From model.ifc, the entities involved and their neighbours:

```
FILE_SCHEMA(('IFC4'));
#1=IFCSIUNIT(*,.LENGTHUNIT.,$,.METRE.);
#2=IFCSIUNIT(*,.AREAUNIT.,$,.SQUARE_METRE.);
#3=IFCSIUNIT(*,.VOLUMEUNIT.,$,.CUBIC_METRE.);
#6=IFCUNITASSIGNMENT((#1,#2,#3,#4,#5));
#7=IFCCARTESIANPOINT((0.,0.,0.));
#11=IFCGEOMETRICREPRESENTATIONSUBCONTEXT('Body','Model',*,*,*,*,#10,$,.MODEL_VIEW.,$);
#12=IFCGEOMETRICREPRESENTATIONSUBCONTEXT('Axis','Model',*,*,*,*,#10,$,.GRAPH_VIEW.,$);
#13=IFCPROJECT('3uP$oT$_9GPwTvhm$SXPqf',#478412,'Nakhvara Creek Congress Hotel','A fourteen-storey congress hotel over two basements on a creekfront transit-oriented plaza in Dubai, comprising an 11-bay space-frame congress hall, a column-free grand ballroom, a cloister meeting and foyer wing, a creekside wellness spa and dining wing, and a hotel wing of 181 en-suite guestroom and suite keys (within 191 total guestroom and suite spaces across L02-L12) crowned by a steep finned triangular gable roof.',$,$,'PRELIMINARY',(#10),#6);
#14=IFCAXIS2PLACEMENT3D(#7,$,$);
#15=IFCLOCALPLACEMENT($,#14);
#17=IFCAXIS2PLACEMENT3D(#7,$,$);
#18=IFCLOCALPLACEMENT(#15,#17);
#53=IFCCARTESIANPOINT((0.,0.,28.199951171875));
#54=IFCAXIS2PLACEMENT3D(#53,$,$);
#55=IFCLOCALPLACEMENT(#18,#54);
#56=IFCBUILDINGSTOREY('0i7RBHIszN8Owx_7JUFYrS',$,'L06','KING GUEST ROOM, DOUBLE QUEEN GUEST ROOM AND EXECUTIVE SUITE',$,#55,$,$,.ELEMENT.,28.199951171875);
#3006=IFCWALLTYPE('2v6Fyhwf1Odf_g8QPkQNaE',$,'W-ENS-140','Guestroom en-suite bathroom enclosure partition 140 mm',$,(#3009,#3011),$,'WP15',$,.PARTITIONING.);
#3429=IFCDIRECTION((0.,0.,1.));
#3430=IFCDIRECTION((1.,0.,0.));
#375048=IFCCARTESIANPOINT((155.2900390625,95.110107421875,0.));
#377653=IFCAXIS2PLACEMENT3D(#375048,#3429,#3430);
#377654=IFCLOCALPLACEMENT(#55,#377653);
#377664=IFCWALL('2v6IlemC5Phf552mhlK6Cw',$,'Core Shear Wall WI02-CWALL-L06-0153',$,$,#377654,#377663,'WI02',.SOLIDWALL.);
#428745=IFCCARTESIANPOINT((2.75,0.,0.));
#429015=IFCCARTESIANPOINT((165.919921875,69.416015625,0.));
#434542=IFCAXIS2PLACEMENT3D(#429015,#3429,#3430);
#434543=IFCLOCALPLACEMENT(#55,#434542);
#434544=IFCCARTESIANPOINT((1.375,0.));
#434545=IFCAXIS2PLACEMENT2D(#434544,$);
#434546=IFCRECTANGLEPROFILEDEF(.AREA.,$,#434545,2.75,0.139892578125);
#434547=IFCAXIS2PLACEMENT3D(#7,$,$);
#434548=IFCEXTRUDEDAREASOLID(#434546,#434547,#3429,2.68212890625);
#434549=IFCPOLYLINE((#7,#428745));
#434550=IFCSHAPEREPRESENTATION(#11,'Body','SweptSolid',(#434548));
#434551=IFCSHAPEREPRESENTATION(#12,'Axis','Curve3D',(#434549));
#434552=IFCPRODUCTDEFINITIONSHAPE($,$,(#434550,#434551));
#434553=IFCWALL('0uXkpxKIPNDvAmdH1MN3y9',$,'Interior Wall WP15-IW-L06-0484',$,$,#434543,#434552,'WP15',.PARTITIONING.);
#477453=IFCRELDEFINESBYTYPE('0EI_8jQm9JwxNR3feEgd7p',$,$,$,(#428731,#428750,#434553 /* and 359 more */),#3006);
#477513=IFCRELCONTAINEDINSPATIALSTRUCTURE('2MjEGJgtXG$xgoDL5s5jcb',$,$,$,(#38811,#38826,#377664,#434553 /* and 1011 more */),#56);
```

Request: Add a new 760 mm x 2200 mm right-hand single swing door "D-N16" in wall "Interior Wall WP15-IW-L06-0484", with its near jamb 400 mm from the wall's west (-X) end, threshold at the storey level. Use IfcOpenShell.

```python
import numpy as np
import ifcopenshell
import ifcopenshell.api.feature
import ifcopenshell.api.geometry
import ifcopenshell.api.root
import ifcopenshell.api.spatial
import ifcopenshell.geom
import ifcopenshell.util.element
import ifcopenshell.util.placement
import ifcopenshell.util.representation
import ifcopenshell.util.shape
import ifcopenshell.util.unit

model = ifcopenshell.open("model.ifc")
unit_scale = ifcopenshell.util.unit.calculate_unit_scale(model)
settings = ifcopenshell.geom.settings()


def volume(element):
    """Net volume in cubic metres, openings subtracted."""
    shape = ifcopenshell.geom.create_shape(settings, element)
    return ifcopenshell.util.shape.get_volume(shape.geometry)


wall = model.by_guid("0uXkpxKIPNDvAmdH1MN3y9")
storey = ifcopenshell.util.element.get_container(wall, ifc_class="IfcBuildingStorey")
context = ifcopenshell.util.representation.get_context(model, "Model", "Body", "MODEL_VIEW")
before = volume(wall)

width, height, from_end, sill = 0.76, 2.2, 0.4, 0.0  # metres

# The wall runs along its own X axis, and the end named is its -X end.
wall_shape = ifcopenshell.geom.create_shape(settings, wall)
x, y, z = ifcopenshell.util.shape.get_vertices(wall_shape.geometry).T
start = x.min() + from_end
face, thickness = float(y.min()), float(y.max() - y.min())
wall_matrix = ifcopenshell.util.placement.get_local_placement(wall.ObjectPlacement)
level = ifcopenshell.util.placement.get_local_placement(storey.ObjectPlacement)[2, 3]


def in_wall(x, y):
    """Placement at x, y metres in the wall's axes, at sill height."""
    matrix = wall_matrix.copy()
    matrix[:, 3] = wall_matrix @ np.array([x / unit_scale, y / unit_scale, 0.0, 1.0])
    matrix[2, 3] = level + sill / unit_scale
    return matrix


# Opening: a box that overshoots both wall faces by 50 mm.
opening = ifcopenshell.api.root.create_entity(model, ifc_class="IfcOpeningElement", predefined_type="OPENING")
box = ifcopenshell.api.geometry.add_wall_representation(
    model, context=context, length=width, height=height, thickness=thickness + 0.1
)
ifcopenshell.api.geometry.assign_representation(model, product=opening, representation=box)
ifcopenshell.api.geometry.edit_object_placement(model, product=opening, matrix=in_wall(start, face - 0.05), is_si=False)
ifcopenshell.api.feature.add_feature(model, feature=opening, element=wall)

door = ifcopenshell.api.root.create_entity(model, ifc_class="IfcDoor", name="D-N16", predefined_type="DOOR")
door.OverallWidth, door.OverallHeight = width / unit_scale, height / unit_scale
door.OperationType = "SINGLE_SWING_RIGHT"
body = ifcopenshell.api.geometry.add_door_representation(
    model,
    context=context,
    overall_width=door.OverallWidth,
    overall_height=door.OverallHeight,
    operation_type="SINGLE_SWING_RIGHT",
    lining_properties={"LiningDepth": thickness / unit_scale, "ThresholdDepth": thickness / unit_scale},
)
ifcopenshell.api.geometry.assign_representation(model, product=door, representation=body)
ifcopenshell.api.spatial.assign_container(model, products=[door], relating_structure=storey)
ifcopenshell.api.feature.add_filling(model, opening=opening, element=door)

# The lining spans the wall, so the door starts at the wall face.
ifcopenshell.api.geometry.edit_object_placement(model, product=door, matrix=in_wall(start, face), is_si=False)

after = volume(wall)

print(f"wall volume {before:.3f} -> {after:.3f} m3")

model.write("model-out.ifc")
```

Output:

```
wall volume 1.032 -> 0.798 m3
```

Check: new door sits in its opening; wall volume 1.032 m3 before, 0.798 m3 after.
